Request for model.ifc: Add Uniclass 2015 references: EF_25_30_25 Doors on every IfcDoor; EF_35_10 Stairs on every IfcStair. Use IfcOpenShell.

First a look at what the model holds.

```python
import ifcopenshell

model = ifcopenshell.open("model.ifc")
print(model.schema)
print("classifications:", [c.Name for c in model.by_type("IfcClassification")])
for ifc_class in ("IfcDoor", "IfcRoof", "IfcStair", "IfcWall", "IfcWindow"):
    print(ifc_class, len(model.by_type(ifc_class)))
```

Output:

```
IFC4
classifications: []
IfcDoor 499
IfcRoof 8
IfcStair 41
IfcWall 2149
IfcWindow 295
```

```python
import ifcopenshell
import ifcopenshell.api.classification

model = ifcopenshell.open("model.ifc")

system = ifcopenshell.api.classification.add_classification(model, classification="Uniclass 2015")

codes = {
    "IfcDoor": ("EF_25_30_25", "Doors"),
    "IfcStair": ("EF_35_10", "Stairs"),
}
for ifc_class, (code, name) in codes.items():
    products = model.by_type(ifc_class)
    ifcopenshell.api.classification.add_reference(
        model, products=products, classification=system, identification=code, name=name
    )
    print(code, len(products))

model.write("model_v2.ifc")
```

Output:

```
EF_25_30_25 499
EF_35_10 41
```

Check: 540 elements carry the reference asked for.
